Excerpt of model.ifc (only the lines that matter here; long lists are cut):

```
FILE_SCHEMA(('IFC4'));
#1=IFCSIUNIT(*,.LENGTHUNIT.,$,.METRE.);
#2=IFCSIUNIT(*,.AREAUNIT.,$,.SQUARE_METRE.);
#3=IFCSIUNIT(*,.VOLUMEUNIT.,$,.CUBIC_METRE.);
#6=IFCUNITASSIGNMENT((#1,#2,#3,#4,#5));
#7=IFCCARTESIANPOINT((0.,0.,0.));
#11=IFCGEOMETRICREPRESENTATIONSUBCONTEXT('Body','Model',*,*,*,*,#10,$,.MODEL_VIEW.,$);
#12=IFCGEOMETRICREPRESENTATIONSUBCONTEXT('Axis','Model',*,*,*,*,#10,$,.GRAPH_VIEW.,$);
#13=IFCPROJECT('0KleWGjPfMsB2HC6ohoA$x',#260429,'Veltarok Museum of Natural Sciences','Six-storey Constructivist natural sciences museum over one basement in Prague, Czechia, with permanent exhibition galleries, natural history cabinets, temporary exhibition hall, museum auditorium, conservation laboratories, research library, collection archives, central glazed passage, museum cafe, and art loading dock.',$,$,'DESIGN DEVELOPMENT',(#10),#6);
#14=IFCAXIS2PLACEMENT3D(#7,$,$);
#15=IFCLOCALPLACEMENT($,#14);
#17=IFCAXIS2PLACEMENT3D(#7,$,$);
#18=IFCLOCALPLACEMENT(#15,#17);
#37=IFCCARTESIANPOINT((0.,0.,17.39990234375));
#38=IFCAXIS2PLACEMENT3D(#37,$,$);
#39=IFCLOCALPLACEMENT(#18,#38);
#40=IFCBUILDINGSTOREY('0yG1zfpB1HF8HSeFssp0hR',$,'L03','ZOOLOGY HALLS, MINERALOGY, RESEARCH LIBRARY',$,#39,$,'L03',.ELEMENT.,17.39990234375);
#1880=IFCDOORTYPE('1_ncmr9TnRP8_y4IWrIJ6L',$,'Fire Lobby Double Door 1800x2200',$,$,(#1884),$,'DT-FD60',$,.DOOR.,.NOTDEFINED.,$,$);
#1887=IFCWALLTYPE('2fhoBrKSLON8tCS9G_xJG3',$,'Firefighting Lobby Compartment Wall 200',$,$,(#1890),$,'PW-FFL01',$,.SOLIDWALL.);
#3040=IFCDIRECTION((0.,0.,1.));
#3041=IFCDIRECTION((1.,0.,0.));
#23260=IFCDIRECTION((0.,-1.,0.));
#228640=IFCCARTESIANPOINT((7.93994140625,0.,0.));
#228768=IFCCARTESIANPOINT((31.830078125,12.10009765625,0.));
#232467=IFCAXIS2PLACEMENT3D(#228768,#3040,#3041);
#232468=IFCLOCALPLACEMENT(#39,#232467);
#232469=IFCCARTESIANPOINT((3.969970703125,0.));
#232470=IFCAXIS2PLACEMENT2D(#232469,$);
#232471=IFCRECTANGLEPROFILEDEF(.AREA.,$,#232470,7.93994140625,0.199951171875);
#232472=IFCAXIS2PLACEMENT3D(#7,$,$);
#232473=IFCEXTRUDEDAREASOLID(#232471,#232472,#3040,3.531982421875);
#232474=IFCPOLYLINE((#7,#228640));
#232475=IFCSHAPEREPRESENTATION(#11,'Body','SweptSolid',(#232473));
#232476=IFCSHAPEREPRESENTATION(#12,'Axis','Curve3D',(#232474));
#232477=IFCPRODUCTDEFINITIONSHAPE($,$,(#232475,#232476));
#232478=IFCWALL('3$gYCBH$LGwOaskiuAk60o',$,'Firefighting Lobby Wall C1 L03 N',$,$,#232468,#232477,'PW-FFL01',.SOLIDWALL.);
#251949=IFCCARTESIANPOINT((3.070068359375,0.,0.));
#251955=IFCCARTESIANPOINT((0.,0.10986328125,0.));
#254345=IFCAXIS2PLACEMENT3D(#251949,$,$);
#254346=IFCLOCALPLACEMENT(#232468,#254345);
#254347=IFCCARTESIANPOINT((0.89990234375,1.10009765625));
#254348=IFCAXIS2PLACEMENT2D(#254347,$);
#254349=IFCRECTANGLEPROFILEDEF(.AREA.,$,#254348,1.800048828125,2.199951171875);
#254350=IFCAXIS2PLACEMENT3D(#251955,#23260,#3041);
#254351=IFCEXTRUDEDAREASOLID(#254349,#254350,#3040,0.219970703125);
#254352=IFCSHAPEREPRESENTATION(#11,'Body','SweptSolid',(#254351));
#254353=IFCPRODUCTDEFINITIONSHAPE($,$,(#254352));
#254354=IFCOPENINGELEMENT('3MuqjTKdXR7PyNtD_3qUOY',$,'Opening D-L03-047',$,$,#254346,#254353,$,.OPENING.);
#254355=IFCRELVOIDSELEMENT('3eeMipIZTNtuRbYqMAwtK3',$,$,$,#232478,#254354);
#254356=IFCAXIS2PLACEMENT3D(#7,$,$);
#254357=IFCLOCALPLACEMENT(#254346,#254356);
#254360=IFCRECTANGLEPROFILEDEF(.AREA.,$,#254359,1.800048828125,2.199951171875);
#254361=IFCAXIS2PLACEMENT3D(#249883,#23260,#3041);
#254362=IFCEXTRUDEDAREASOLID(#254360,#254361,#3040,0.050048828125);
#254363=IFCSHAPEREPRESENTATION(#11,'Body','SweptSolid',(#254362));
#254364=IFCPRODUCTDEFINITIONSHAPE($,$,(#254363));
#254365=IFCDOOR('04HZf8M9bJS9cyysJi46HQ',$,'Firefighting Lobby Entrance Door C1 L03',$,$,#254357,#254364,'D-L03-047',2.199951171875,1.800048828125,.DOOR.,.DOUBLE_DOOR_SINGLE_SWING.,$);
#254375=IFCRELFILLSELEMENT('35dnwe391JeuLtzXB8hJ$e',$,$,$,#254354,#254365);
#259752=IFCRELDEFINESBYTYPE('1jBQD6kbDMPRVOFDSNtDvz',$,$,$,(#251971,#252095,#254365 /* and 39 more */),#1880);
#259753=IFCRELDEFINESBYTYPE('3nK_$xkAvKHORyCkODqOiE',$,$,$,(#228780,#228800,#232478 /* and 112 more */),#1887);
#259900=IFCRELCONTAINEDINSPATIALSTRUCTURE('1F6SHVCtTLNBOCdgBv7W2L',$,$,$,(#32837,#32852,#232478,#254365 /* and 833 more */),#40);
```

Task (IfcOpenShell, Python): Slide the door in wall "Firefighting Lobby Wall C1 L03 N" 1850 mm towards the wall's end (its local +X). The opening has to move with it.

```python
import ifcopenshell
import ifcopenshell.api.geometry
import ifcopenshell.util.placement

model = ifcopenshell.open("model.ifc")

door = model.by_guid("04HZf8M9bJS9cyysJi46HQ")
opening = door.FillsVoids[0].RelatingOpeningElement
wall = opening.VoidsElements[0].RelatingBuildingElement

wall_matrix = ifcopenshell.util.placement.get_local_placement(wall.ObjectPlacement)
shift = wall_matrix[:3, 0] * 1.85
before = ifcopenshell.util.placement.get_local_placement(door.ObjectPlacement)[:3, 3].copy()

# The door is placed relative to its opening, so it follows when the opening moves.
matrix = ifcopenshell.util.placement.get_local_placement(opening.ObjectPlacement)
matrix[:3, 3] += shift
ifcopenshell.api.geometry.edit_object_placement(
    model, product=opening, matrix=matrix, is_si=False, should_transform_children=True
)

after = ifcopenshell.util.placement.get_local_placement(door.ObjectPlacement)[:3, 3]
print("door moved by", (after - before).round(3) + 0.0)

model.write("model_edited.ifc")
```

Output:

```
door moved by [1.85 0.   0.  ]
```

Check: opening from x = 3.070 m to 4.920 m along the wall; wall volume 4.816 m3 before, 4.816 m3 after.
